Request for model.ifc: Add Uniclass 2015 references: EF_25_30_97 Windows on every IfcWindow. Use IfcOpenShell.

First a look at what the model holds.

```python
import ifcopenshell

model = ifcopenshell.open("model.ifc")
print(model.schema)
print("classifications:", [c.Name for c in model.by_type("IfcClassification")])
for ifc_class in ("IfcDoor", "IfcRoof", "IfcStair", "IfcWall", "IfcWindow"):
    print(ifc_class, len(model.by_type(ifc_class)))
```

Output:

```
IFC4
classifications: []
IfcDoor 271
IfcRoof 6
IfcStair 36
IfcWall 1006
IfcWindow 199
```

```python
import ifcopenshell
import ifcopenshell.api.classification

model = ifcopenshell.open("model.ifc")

system = ifcopenshell.api.classification.add_classification(model, classification="Uniclass 2015")

codes = {
    "IfcWindow": ("EF_25_30_97", "Windows"),
}
for ifc_class, (code, name) in codes.items():
    products = model.by_type(ifc_class)
    ifcopenshell.api.classification.add_reference(
        model, products=products, classification=system, identification=code, name=name
    )
    print(code, len(products))

model.write("model_rev.ifc")
```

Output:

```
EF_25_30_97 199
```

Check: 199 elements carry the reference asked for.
